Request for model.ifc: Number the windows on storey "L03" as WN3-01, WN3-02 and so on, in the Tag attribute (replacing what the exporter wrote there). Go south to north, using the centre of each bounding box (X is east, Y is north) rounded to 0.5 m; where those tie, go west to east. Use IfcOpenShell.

First a look at what the model holds.

```python
import ifcopenshell
import ifcopenshell.util.element
import ifcopenshell.util.placement

model = ifcopenshell.open("model.ifc")
print(model.schema)
storey = next(s for s in model.by_type("IfcBuildingStorey") if s.Name == "L03")
windows = [e for e in ifcopenshell.util.element.get_decomposition(storey) if e.is_a("IfcWindow")]
for e in sorted(windows, key=lambda e: e.id()):
    origin = ifcopenshell.util.placement.get_local_placement(e.ObjectPlacement)[:3, 3]
    print(e.id(), e.Tag, e.Name, origin.round(2) + 0.0, sep=" | ")
```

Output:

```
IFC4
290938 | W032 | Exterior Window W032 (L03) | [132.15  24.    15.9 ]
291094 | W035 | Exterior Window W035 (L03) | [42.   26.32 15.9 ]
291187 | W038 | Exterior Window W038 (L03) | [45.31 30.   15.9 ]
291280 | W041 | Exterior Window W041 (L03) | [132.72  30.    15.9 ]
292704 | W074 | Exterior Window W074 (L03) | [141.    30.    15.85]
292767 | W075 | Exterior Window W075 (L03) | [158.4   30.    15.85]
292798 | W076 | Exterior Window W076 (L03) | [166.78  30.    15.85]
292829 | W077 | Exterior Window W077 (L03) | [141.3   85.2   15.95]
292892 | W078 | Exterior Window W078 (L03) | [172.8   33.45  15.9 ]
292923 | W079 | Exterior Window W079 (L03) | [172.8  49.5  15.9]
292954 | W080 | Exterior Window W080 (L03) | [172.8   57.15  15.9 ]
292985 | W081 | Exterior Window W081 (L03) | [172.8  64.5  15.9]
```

```python
import ifcopenshell
import ifcopenshell.geom
import ifcopenshell.util.element
import ifcopenshell.util.shape

model = ifcopenshell.open("model.ifc")
settings = ifcopenshell.geom.settings()
settings.set("use-world-coords", True)


def centre(element):
    shape = ifcopenshell.geom.create_shape(settings, element)
    return ifcopenshell.util.shape.get_bbox_centroid(shape.geometry)


storey = next(s for s in model.by_type("IfcBuildingStorey") if s.Name == "L03")
windows = [e for e in ifcopenshell.util.element.get_decomposition(storey) if e.is_a("IfcWindow")]

# Insertion points can sit at a corner or the storey origin, so sort by the geometry (in metres).
centres = {e: centre(e) for e in windows}
windows.sort(key=lambda e: (round(centres[e][1] / 0.5), centres[e][0]))

for i, e in enumerate(windows, start=1):
    number = f"WN3-{i:02d}"
    e.Tag = number
    print(e.id(), number)

model.write("model_updated.ifc")
```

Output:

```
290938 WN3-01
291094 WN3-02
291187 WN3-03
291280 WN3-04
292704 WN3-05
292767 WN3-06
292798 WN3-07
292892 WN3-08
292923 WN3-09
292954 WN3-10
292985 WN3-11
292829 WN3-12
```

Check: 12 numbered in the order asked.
